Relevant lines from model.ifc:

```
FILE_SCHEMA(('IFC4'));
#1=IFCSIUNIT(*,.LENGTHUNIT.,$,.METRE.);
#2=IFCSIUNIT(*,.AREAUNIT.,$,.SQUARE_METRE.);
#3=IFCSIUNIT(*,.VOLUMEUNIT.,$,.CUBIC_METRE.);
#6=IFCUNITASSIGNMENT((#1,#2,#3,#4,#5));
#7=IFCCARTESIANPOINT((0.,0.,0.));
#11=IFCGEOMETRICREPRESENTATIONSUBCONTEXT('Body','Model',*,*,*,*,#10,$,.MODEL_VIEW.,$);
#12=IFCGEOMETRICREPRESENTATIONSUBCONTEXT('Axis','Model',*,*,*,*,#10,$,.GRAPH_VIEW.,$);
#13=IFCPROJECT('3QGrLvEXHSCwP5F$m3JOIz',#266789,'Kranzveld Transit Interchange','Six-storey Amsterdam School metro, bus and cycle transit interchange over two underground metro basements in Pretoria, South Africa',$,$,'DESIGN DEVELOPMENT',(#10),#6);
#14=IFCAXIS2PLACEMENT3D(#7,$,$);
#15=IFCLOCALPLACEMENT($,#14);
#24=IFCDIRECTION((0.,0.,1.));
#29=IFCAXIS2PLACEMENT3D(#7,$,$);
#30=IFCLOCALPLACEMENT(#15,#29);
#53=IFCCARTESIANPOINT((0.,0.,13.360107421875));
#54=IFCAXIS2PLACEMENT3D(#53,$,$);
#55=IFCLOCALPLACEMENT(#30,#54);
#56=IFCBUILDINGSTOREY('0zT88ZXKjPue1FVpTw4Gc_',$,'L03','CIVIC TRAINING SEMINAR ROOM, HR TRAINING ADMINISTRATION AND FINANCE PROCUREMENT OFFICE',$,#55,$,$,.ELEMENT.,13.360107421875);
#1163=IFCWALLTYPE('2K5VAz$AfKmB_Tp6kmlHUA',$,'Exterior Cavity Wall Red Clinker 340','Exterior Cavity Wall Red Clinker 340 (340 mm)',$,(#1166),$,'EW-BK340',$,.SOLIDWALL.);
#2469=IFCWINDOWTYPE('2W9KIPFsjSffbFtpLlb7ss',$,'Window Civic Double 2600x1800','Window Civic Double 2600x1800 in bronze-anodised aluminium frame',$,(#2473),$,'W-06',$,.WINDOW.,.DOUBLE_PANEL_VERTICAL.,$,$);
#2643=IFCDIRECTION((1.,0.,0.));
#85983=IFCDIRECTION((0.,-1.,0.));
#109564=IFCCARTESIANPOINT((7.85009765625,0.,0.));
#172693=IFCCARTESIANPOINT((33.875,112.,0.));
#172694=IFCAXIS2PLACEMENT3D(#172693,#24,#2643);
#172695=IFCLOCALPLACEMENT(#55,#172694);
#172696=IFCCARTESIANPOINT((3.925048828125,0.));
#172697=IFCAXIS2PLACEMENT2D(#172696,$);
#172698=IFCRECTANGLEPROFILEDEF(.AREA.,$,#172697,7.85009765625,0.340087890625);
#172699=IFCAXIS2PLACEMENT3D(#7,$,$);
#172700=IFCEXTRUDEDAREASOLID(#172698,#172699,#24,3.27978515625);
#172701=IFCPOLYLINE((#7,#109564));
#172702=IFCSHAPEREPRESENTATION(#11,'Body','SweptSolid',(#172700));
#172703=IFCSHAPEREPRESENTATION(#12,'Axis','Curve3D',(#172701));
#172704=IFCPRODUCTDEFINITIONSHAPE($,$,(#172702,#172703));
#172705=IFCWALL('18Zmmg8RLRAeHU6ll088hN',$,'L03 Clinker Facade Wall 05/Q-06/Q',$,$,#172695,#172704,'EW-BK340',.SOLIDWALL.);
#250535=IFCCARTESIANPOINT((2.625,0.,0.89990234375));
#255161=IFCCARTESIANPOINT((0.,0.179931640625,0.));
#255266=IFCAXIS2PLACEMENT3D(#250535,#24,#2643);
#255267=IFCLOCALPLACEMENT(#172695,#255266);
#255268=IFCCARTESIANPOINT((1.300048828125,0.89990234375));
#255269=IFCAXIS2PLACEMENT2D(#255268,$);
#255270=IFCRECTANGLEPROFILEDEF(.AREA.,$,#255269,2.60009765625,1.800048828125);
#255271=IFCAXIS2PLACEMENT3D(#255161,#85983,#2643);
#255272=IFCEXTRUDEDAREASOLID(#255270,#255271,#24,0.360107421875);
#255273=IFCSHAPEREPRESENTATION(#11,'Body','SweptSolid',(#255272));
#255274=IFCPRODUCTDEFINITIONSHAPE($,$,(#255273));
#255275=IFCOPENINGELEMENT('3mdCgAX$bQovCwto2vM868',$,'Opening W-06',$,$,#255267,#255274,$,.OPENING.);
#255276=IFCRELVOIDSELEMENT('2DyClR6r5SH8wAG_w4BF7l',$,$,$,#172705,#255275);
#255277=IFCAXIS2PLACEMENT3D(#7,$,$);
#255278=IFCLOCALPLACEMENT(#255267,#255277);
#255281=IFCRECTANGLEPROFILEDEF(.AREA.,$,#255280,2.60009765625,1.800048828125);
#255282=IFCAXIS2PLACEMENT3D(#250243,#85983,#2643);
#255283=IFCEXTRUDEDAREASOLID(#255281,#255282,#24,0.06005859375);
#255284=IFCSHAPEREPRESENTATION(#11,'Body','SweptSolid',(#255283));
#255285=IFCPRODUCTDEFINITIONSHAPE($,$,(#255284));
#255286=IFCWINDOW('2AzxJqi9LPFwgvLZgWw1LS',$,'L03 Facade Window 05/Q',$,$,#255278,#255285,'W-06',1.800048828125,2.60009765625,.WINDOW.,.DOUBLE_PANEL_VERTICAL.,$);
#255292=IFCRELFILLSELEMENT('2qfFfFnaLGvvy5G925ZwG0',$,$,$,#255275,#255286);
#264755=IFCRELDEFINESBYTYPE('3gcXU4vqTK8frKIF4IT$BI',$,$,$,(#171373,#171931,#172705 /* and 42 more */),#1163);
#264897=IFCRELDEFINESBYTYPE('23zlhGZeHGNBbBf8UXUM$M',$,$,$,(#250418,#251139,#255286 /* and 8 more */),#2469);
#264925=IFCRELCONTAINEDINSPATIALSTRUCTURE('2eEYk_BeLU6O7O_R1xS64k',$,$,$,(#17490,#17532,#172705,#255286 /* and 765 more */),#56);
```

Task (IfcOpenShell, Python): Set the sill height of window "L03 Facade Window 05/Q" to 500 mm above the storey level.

```python
import numpy as np
import ifcopenshell
import ifcopenshell.api.geometry
import ifcopenshell.geom
import ifcopenshell.util.element
import ifcopenshell.util.placement
import ifcopenshell.util.shape
import ifcopenshell.util.unit

model = ifcopenshell.open("model.ifc")
unit_scale = ifcopenshell.util.unit.calculate_unit_scale(model)

window = model.by_id(255286)
opening = window.FillsVoids[0].RelatingOpeningElement
storey = ifcopenshell.util.element.get_container(window, ifc_class="IfcBuildingStorey")
level = ifcopenshell.util.placement.get_local_placement(storey.ObjectPlacement)[2, 3]

# The opening's origin need not be at the sill, so measure its lowest point.
shape = ifcopenshell.geom.create_shape(ifcopenshell.geom.settings(), opening)
bottom = ifcopenshell.util.shape.get_shape_bottom_elevation(shape, shape.geometry) / unit_scale
dz = level + 0.5 / unit_scale - bottom

shift = np.array([0.0, 0.0, dz])
# The window is placed relative to its opening, so it follows when the opening moves.
matrix = ifcopenshell.util.placement.get_local_placement(opening.ObjectPlacement)
matrix[:3, 3] += shift
ifcopenshell.api.geometry.edit_object_placement(
    model, product=opening, matrix=matrix, is_si=False, should_transform_children=True
)

print(f"moved by {dz * unit_scale:+.3f} m")

model.write("model-out.ifc")
```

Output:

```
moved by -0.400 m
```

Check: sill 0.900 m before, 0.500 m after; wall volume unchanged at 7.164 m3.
